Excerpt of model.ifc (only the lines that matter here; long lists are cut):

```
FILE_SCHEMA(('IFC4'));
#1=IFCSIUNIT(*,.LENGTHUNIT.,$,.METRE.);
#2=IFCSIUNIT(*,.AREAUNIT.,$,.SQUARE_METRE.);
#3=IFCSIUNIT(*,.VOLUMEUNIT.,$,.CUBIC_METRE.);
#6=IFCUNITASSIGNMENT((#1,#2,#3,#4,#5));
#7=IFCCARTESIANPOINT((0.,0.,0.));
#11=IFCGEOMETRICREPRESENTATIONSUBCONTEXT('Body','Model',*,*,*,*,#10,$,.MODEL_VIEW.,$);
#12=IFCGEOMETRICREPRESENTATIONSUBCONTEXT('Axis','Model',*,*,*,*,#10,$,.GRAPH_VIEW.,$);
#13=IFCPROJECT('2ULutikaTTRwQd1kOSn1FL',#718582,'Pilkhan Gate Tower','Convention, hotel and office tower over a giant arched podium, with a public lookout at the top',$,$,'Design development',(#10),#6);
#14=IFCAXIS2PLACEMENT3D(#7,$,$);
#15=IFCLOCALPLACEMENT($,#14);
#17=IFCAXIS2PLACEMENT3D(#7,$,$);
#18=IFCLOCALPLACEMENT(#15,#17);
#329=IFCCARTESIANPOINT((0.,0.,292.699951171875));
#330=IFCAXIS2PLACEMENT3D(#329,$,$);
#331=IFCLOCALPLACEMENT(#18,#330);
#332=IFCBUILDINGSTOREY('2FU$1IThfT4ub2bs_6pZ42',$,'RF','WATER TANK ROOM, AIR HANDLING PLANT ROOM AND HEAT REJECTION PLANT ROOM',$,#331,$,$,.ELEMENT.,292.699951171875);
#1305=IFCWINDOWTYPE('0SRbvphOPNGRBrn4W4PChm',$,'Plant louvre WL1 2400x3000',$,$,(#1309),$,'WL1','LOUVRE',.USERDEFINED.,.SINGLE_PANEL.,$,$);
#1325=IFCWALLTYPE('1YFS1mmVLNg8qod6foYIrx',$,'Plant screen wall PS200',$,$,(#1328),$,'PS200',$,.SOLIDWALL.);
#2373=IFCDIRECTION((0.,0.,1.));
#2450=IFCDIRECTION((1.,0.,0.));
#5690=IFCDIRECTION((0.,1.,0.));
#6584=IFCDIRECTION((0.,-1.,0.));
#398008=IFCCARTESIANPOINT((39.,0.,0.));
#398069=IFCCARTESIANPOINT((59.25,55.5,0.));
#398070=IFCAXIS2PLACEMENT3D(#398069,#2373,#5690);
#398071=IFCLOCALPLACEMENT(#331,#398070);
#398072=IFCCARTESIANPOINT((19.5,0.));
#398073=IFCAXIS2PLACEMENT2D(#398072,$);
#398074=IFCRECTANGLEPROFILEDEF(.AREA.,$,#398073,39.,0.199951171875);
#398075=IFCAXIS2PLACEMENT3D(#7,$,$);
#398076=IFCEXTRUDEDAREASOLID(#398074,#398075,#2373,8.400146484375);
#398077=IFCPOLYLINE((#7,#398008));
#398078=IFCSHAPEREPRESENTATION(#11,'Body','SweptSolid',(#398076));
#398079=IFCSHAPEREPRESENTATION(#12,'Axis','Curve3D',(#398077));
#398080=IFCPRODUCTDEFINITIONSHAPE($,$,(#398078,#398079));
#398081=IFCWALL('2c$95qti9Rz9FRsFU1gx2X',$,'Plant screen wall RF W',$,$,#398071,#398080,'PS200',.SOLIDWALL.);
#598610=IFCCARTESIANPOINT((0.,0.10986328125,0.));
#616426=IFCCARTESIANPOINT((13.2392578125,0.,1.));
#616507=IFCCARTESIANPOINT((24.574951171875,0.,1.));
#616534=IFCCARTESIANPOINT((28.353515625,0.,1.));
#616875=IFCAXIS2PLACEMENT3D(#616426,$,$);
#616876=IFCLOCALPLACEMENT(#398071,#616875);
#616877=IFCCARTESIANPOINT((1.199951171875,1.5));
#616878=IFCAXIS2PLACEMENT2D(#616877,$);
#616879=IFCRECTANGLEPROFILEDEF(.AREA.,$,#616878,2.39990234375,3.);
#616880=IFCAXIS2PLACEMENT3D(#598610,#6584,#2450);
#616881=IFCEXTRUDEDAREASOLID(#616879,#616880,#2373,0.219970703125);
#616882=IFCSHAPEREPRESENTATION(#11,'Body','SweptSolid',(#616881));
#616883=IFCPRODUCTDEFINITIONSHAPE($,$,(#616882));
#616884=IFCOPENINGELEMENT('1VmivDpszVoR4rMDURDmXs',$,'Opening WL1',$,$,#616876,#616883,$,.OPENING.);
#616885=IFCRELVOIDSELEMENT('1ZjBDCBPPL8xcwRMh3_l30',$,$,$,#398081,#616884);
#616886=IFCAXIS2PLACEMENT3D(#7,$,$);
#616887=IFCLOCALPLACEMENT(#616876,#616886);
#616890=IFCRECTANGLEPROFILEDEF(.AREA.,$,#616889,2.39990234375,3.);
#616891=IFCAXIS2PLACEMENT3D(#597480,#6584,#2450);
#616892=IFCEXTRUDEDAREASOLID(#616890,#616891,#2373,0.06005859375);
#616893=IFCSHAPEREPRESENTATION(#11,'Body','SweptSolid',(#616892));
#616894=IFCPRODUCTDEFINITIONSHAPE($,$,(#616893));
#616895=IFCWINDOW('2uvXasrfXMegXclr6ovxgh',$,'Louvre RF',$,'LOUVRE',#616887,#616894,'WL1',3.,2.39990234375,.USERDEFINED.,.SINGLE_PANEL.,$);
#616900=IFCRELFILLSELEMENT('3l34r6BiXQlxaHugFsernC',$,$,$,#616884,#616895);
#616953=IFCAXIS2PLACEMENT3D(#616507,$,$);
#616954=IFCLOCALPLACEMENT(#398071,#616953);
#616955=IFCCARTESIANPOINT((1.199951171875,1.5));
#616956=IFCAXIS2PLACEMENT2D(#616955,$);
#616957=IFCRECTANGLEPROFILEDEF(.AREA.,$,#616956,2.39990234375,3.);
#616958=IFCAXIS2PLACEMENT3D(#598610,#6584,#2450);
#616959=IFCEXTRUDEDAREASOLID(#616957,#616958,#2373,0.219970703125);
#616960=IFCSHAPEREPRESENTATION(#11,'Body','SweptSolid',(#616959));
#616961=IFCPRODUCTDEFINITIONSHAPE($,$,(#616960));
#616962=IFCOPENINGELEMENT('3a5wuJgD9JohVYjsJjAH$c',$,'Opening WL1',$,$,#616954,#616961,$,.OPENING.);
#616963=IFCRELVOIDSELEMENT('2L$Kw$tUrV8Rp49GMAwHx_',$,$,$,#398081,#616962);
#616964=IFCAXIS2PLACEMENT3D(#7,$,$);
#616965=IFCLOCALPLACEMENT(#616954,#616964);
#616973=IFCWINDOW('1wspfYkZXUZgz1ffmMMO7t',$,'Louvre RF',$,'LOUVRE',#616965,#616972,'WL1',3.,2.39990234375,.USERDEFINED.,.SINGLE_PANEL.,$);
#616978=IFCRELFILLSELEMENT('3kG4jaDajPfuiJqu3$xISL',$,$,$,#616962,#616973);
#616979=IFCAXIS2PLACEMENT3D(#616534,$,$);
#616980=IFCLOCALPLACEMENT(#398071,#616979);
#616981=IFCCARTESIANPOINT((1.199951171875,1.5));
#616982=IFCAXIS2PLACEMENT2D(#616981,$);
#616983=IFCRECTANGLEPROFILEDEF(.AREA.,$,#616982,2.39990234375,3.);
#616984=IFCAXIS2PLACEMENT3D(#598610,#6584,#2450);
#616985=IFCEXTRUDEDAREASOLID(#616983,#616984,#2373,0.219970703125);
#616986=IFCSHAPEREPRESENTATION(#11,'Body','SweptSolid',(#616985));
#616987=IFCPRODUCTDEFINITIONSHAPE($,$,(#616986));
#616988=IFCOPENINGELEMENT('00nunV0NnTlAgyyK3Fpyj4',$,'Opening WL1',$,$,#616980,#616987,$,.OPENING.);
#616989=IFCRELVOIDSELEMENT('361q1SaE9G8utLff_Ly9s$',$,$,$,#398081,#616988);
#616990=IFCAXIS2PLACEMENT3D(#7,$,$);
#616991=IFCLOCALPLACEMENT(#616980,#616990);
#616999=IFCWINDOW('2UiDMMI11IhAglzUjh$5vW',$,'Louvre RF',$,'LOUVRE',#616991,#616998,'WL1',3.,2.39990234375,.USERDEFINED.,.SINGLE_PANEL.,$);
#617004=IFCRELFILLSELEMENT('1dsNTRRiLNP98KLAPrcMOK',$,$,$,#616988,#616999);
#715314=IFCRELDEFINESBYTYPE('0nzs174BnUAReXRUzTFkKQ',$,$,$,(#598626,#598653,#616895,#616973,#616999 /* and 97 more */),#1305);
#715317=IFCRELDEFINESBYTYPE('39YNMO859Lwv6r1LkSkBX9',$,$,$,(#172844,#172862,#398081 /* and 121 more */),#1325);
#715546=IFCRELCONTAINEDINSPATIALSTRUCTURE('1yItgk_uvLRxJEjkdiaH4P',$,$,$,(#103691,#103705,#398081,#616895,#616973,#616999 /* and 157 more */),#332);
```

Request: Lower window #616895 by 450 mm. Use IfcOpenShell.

```python
import numpy as np
import ifcopenshell
import ifcopenshell.api.geometry
import ifcopenshell.util.placement
import ifcopenshell.util.unit

model = ifcopenshell.open("model.ifc")
unit_scale = ifcopenshell.util.unit.calculate_unit_scale(model)

window = model.by_guid("2uvXasrfXMegXclr6ovxgh")
opening = window.FillsVoids[0].RelatingOpeningElement
dz = -0.45

shift = np.array([0.0, 0.0, dz])
# The window is placed relative to its opening, so it follows when the opening moves.
matrix = ifcopenshell.util.placement.get_local_placement(opening.ObjectPlacement)
matrix[:3, 3] += shift
ifcopenshell.api.geometry.edit_object_placement(
    model, product=opening, matrix=matrix, is_si=False, should_transform_children=True
)

print(f"moved by {dz * unit_scale:+.3f} m")

model.write("model_v2.ifc")
```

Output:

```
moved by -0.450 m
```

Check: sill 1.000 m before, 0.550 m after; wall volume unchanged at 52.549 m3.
